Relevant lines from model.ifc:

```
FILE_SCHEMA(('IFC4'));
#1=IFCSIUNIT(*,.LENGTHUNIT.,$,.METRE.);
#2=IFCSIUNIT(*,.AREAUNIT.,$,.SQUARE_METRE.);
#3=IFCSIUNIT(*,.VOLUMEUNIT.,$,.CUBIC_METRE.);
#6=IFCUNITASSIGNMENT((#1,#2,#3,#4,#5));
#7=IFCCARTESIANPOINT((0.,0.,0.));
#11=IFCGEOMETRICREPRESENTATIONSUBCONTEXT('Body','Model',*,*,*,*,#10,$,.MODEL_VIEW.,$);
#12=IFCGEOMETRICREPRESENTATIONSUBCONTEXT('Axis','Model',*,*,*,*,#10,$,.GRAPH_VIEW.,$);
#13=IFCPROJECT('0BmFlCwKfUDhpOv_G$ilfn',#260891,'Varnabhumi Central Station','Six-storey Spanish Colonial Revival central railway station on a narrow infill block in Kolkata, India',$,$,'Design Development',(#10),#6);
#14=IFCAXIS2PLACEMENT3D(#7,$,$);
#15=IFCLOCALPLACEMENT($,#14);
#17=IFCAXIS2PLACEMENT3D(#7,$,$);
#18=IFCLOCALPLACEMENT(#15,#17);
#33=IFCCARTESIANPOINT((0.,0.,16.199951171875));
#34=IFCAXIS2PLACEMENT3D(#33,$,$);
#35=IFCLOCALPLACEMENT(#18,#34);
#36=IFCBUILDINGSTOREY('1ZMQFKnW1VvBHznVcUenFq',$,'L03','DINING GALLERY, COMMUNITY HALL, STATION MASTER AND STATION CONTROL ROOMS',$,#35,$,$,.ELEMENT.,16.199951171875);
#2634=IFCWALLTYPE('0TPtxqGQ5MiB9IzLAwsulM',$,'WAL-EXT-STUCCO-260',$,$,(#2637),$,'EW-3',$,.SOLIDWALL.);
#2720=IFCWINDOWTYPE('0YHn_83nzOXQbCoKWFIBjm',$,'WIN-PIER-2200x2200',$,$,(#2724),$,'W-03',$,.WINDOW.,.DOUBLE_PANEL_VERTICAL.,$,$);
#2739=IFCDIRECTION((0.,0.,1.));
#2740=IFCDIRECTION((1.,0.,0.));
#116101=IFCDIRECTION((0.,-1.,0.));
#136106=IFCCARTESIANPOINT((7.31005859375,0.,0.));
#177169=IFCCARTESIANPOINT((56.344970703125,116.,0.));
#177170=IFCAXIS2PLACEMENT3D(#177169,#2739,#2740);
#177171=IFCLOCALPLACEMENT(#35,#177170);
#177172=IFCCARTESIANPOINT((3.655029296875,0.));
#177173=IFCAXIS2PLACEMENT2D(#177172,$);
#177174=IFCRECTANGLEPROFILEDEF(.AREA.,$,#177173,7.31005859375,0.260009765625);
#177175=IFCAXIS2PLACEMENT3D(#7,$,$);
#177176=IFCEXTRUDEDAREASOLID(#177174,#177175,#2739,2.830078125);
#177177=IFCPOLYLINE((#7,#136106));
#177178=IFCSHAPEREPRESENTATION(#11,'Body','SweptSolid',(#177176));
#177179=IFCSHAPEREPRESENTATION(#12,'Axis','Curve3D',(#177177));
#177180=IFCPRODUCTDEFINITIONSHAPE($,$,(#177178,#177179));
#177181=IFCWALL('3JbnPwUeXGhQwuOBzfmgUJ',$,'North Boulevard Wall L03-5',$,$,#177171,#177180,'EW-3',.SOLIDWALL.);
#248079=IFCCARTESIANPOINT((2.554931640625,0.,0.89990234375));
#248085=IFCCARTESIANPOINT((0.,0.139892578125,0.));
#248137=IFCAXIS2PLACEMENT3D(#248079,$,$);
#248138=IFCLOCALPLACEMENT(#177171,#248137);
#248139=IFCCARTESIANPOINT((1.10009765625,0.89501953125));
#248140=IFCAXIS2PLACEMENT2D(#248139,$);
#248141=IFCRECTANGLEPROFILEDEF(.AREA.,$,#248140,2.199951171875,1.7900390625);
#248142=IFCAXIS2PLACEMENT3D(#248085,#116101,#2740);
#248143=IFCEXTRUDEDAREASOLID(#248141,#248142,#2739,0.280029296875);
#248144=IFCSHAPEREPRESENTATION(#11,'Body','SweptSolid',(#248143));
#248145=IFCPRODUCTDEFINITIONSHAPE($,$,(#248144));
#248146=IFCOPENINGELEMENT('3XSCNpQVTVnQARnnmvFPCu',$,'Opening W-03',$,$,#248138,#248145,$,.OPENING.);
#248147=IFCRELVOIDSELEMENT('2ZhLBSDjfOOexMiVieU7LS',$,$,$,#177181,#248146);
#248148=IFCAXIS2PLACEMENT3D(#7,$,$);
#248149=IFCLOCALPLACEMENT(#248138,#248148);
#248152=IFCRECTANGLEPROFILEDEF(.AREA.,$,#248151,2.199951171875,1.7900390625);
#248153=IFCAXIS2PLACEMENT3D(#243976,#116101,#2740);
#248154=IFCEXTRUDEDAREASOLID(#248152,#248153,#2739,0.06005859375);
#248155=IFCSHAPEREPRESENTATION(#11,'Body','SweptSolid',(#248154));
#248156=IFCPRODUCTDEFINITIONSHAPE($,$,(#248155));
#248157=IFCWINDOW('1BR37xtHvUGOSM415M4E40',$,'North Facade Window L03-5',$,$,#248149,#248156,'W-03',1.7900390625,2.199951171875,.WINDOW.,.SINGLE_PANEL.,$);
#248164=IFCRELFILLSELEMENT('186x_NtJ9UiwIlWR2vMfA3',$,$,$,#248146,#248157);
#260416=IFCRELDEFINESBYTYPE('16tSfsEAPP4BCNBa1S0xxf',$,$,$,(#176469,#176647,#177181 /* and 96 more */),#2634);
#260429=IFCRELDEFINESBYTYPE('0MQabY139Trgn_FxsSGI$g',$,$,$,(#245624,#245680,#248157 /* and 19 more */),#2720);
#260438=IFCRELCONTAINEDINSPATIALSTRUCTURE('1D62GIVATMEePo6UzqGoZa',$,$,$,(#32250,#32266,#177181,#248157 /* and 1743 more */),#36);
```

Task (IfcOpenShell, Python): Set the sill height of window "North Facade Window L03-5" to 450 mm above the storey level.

```python
import numpy as np
import ifcopenshell
import ifcopenshell.api.geometry
import ifcopenshell.geom
import ifcopenshell.util.element
import ifcopenshell.util.placement
import ifcopenshell.util.shape
import ifcopenshell.util.unit

model = ifcopenshell.open("model.ifc")
unit_scale = ifcopenshell.util.unit.calculate_unit_scale(model)

window = model.by_id(248157)
opening = window.FillsVoids[0].RelatingOpeningElement
storey = ifcopenshell.util.element.get_container(window, ifc_class="IfcBuildingStorey")
level = ifcopenshell.util.placement.get_local_placement(storey.ObjectPlacement)[2, 3]

# The opening's origin need not be at the sill, so measure its lowest point.
shape = ifcopenshell.geom.create_shape(ifcopenshell.geom.settings(), opening)
bottom = ifcopenshell.util.shape.get_shape_bottom_elevation(shape, shape.geometry) / unit_scale
dz = level + 0.45 - bottom

shift = np.array([0.0, 0.0, dz])
# The window is placed relative to its opening, so it follows when the opening moves.
matrix = ifcopenshell.util.placement.get_local_placement(opening.ObjectPlacement)
matrix[:3, 3] += shift
ifcopenshell.api.geometry.edit_object_placement(
    model, product=opening, matrix=matrix, is_si=False, should_transform_children=True
)

print(f"moved by {dz * unit_scale:+.3f} m")

model.write("model-out.ifc")
```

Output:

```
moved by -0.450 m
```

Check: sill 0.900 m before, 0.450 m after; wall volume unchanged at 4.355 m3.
